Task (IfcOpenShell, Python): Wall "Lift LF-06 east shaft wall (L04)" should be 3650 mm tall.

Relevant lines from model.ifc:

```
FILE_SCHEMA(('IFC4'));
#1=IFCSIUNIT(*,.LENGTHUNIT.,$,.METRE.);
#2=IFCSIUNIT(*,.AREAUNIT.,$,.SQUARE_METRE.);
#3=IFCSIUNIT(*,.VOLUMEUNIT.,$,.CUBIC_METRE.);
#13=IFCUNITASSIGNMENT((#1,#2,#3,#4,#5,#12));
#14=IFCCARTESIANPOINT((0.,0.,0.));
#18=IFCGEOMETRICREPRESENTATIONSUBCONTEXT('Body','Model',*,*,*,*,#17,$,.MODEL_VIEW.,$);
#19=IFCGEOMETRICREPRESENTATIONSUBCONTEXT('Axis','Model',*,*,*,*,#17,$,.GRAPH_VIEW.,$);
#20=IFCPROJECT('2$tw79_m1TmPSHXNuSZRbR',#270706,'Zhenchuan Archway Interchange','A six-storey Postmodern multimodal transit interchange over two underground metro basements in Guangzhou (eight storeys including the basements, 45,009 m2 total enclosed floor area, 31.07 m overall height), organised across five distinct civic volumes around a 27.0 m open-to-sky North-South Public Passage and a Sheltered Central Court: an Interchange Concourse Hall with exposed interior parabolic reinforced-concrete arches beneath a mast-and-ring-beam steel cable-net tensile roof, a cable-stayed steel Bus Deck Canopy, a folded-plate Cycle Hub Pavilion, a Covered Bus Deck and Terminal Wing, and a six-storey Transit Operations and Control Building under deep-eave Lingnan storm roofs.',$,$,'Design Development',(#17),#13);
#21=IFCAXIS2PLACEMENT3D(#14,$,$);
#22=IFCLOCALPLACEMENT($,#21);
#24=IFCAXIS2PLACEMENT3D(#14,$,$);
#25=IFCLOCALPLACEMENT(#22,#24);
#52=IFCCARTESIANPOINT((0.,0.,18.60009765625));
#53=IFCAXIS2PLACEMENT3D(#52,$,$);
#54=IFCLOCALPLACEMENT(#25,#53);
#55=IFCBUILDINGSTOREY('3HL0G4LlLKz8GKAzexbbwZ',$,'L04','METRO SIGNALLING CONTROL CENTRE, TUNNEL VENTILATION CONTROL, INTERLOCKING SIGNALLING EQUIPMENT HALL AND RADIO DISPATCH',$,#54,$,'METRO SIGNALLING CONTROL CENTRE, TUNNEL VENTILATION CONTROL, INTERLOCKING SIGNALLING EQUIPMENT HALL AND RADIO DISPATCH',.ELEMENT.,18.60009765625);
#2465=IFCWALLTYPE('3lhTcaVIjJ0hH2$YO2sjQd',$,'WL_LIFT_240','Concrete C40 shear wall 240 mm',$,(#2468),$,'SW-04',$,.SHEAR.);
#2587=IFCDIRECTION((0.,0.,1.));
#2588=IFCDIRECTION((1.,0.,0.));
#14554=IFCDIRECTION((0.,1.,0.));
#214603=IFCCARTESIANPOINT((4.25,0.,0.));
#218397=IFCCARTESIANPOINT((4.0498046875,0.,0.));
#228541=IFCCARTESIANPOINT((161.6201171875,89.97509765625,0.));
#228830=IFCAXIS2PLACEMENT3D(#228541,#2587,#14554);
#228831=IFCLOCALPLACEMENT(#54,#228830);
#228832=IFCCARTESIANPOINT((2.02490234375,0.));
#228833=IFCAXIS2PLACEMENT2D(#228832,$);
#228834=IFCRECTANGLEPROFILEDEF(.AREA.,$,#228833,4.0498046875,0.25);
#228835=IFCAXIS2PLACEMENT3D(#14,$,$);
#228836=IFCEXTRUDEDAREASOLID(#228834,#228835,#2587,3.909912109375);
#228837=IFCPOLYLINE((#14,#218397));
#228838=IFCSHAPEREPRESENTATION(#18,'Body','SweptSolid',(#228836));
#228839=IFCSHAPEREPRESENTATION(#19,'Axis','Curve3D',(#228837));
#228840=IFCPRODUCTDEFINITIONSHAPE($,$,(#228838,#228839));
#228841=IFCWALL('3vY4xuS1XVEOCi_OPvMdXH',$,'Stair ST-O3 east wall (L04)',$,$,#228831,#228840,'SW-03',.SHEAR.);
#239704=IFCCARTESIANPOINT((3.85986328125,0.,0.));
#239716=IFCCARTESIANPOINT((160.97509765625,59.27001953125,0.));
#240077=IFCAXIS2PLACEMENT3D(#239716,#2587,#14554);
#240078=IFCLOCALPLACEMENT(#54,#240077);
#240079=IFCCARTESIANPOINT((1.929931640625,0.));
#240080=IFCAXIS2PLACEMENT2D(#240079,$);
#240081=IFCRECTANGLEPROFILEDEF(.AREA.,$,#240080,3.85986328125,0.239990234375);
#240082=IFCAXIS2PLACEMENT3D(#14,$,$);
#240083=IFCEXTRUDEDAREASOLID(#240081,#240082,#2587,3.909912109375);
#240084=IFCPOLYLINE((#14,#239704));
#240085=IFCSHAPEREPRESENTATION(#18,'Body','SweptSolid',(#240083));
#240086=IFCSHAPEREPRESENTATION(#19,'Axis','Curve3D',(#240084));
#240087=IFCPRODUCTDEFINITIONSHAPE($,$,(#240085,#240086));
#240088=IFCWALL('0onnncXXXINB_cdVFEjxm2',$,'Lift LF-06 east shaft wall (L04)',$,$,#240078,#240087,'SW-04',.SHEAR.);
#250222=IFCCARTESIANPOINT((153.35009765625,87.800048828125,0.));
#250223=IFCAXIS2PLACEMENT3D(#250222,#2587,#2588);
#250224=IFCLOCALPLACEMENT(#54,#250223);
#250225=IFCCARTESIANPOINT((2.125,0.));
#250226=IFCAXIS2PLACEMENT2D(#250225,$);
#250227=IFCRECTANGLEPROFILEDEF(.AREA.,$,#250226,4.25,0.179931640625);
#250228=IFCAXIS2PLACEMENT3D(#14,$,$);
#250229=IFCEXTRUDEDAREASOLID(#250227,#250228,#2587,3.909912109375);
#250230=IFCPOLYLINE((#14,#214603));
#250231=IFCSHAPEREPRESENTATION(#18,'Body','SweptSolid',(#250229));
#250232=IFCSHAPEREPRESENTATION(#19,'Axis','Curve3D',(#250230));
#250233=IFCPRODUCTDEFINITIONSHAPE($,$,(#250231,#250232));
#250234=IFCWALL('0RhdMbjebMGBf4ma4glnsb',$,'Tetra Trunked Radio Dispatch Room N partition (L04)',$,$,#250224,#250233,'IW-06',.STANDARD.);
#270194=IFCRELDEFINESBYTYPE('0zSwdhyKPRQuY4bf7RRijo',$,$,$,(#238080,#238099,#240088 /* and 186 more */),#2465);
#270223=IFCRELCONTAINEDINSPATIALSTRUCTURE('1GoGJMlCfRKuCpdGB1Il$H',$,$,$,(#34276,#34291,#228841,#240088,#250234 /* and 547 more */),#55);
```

```python
import ifcopenshell
import ifcopenshell.geom
import ifcopenshell.util.representation
import ifcopenshell.util.shape
import ifcopenshell.util.unit

model = ifcopenshell.open("model.ifc")
unit_scale = ifcopenshell.util.unit.calculate_unit_scale(model)
settings = ifcopenshell.geom.settings()


def volume(element):
    """Net volume in cubic metres, openings subtracted."""
    shape = ifcopenshell.geom.create_shape(settings, element)
    return ifcopenshell.util.shape.get_volume(shape.geometry)


wall = model.by_guid("0onnncXXXINB_cdVFEjxm2")
before = volume(wall)

body = ifcopenshell.util.representation.get_representation(wall, "Model", "Body")
solid = body.Items[0]
old_height = solid.Depth
solid.Depth = 3.65 / unit_scale
after = volume(wall)

print(f"height {old_height:g} -> {solid.Depth:g}, volume {before:.3f} -> {after:.3f} m3")

model.write("model_updated.ifc")
```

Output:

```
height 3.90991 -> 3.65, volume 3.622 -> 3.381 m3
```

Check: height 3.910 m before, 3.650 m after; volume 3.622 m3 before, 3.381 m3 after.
